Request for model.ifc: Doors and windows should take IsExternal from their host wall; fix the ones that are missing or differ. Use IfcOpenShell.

First a look at what the model holds.

```python
import ifcopenshell
import ifcopenshell.util.element

model = ifcopenshell.open("model.ifc")
print(model.schema)
seen = {}
for e in model.by_type("IfcDoor") + model.by_type("IfcWindow"):
    if not e.FillsVoids:
        continue
    host = e.FillsVoids[0].RelatingOpeningElement.VoidsElements[0].RelatingBuildingElement
    own = ifcopenshell.util.element.get_pset(e, f"Pset_{e.is_a()[3:].removesuffix('StandardCase')}Common", "IsExternal")
    wall = ifcopenshell.util.element.get_pset(host, "Pset_WallCommon", "IsExternal")
    seen[e.is_a(), own, wall] = seen.get((e.is_a(), own, wall), 0) + 1
for (cls, own, wall), count in sorted(seen.items(), key=str):
    print(count, cls, "IsExternal:", own, "| host wall:", wall)
```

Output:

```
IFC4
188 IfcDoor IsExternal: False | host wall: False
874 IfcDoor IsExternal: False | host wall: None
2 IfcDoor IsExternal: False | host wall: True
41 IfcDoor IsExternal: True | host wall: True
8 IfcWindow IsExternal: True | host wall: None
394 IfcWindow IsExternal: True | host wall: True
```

```python
import ifcopenshell
import ifcopenshell.api.pset
import ifcopenshell.util.element

model = ifcopenshell.open("model.ifc")

count = 0
for ifc_class, pset_name in (("IfcDoor", "Pset_DoorCommon"), ("IfcWindow", "Pset_WindowCommon")):
    for e in model.by_type(ifc_class):
        if not e.FillsVoids:
            continue
        host = e.FillsVoids[0].RelatingOpeningElement.VoidsElements[0].RelatingBuildingElement
        external = ifcopenshell.util.element.get_pset(host, "Pset_WallCommon", "IsExternal")
        if external is None or ifcopenshell.util.element.get_pset(e, pset_name, "IsExternal") == external:
            continue
        pset = ifcopenshell.api.pset.add_pset(model, product=e, name=pset_name)
        ifcopenshell.api.pset.edit_pset(model, pset=pset, properties={"IsExternal": external})
        count += 1

print(count, "updated")

model.write("model_edited.ifc")
```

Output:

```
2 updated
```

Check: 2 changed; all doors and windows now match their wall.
